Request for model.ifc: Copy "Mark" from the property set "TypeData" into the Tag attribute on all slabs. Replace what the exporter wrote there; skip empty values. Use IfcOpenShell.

First a look at what the model holds.

```python
import ifcopenshell
import ifcopenshell.util.element

model = ifcopenshell.open("model.ifc")
print(model.schema)
slabs = model.by_type("IfcSlab")
print(len(slabs), "slabs")
for e in slabs[:8]:
    source = ifcopenshell.util.element.get_pset(e, "TypeData", "Mark")
    target = e.Tag
    print(e.id(), repr(source), repr(target), sep=" | ")
```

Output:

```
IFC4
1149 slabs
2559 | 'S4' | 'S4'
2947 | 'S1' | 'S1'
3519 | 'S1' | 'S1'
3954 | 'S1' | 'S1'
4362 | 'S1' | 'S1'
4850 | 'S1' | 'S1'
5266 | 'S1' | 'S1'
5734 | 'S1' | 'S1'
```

```python
import ifcopenshell
import ifcopenshell.util.element

model = ifcopenshell.open("model.ifc")

count = 0
for e in model.by_type("IfcSlab"):
    value = ifcopenshell.util.element.get_pset(e, "TypeData", "Mark")
    current = e.Tag
    if not value or not value.strip() or current == value:
        continue
    e.Tag = value
    count += 1

print(count, "slabs updated")

model.write("model_updated.ifc")
```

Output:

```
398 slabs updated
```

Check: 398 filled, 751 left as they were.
